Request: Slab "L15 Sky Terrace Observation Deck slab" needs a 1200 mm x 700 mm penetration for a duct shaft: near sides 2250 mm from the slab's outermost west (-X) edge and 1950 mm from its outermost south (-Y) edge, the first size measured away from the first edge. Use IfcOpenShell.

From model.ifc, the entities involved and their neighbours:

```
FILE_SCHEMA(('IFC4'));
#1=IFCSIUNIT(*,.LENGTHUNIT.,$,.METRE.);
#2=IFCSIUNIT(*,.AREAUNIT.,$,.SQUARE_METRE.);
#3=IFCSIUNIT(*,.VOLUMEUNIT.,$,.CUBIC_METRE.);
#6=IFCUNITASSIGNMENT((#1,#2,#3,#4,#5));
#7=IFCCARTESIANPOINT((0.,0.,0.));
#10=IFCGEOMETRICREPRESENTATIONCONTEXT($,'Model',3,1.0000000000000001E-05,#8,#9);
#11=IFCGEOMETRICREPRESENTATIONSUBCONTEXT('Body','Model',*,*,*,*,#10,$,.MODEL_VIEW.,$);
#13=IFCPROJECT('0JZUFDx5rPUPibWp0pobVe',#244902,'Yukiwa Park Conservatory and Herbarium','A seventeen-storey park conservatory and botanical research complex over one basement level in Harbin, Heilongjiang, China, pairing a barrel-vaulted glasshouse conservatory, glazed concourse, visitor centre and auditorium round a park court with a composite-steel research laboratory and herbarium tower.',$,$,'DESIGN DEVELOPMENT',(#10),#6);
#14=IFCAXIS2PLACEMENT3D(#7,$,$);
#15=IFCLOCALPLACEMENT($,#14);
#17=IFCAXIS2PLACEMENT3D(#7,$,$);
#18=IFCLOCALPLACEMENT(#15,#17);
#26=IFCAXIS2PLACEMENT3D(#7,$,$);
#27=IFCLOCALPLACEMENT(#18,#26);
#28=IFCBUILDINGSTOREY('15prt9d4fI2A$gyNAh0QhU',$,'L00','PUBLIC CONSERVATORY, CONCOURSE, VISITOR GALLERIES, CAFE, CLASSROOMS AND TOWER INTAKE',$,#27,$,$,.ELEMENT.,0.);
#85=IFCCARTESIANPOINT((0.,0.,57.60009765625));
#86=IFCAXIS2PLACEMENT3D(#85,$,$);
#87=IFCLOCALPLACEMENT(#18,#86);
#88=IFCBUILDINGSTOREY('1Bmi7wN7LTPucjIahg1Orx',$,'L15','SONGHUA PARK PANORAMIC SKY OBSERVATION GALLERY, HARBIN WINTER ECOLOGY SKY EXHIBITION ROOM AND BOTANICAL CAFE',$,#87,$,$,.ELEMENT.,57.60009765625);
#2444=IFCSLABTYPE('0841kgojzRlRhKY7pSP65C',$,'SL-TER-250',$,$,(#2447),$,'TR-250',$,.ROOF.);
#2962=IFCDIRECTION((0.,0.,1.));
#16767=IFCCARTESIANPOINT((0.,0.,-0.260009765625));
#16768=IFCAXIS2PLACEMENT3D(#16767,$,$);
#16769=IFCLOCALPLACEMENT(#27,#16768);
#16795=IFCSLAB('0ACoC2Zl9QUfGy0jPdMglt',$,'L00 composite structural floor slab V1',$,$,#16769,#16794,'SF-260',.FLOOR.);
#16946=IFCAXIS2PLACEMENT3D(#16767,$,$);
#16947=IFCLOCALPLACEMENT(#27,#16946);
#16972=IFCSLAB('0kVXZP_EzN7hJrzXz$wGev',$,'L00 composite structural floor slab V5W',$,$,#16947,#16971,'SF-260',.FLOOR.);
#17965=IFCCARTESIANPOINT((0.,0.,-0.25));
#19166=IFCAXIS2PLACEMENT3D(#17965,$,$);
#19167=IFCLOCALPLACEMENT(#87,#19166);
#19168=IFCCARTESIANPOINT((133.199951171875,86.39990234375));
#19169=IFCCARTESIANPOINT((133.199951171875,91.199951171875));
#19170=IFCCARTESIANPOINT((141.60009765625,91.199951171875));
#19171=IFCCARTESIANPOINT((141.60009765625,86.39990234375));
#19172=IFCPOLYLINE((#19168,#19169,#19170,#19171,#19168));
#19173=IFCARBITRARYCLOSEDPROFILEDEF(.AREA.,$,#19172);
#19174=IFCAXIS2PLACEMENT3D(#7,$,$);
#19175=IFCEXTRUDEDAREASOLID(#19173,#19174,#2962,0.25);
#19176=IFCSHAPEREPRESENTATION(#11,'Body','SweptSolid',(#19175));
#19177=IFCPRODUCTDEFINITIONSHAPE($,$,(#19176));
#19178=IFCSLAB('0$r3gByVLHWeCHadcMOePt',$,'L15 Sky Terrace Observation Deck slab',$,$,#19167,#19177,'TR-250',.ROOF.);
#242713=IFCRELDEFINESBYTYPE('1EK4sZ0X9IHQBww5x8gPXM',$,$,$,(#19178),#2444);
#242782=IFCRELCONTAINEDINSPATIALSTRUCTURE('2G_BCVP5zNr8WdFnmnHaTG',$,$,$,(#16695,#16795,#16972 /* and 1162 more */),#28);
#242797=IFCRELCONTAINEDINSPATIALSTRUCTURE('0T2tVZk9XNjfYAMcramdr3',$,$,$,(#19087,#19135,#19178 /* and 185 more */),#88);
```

```python
import numpy as np
import ifcopenshell
import ifcopenshell.api.feature
import ifcopenshell.api.geometry
import ifcopenshell.api.root
import ifcopenshell.geom
import ifcopenshell.util.placement
import ifcopenshell.util.representation
import ifcopenshell.util.shape
import ifcopenshell.util.unit

model = ifcopenshell.open("model.ifc")
unit_scale = ifcopenshell.util.unit.calculate_unit_scale(model)
settings = ifcopenshell.geom.settings()


def volume(element):
    """Net volume in cubic metres, openings subtracted."""
    shape = ifcopenshell.geom.create_shape(settings, element)
    return ifcopenshell.util.shape.get_volume(shape.geometry)


slab = model.by_id(19178)
before = volume(slab)

# Extent in the slab's own axes, in metres. The edges named are its -X and -Y sides.
slab_shape = ifcopenshell.geom.create_shape(settings, slab)
vertices = ifcopenshell.util.shape.get_vertices(slab_shape.geometry)
x_min, y_min, bottom = vertices.min(axis=0)
top = vertices[:, 2].max()

opening = ifcopenshell.api.root.create_entity(model, ifc_class="IfcOpeningElement", name="Duct shaft opening", predefined_type="OPENING")
context = ifcopenshell.util.representation.get_context(model, "Model", "Body", "MODEL_VIEW")
width, depth = 1.2, 0.7
outline = [(0.0, 0.0), (width, 0.0), (width, depth), (0.0, depth), (0.0, 0.0)]
# Overshoot both faces by 50 mm so the cut is clean.
shape = ifcopenshell.api.geometry.add_slab_representation(
    model, context=context, depth=top - bottom + 0.1, polyline=outline
)
ifcopenshell.api.geometry.assign_representation(model, product=opening, representation=shape)

matrix = ifcopenshell.util.placement.get_local_placement(slab.ObjectPlacement)
matrix[:, 3] = matrix @ np.append(np.array([x_min + 2.25, y_min + 1.95, bottom - 0.05]) / unit_scale, 1.0)
ifcopenshell.api.geometry.edit_object_placement(model, product=opening, matrix=matrix, is_si=False)
ifcopenshell.api.feature.add_feature(model, feature=opening, element=slab)

after = volume(slab)

print(f"slab volume {before:.3f} -> {after:.3f} m3")

model.write("model_edited.ifc")
```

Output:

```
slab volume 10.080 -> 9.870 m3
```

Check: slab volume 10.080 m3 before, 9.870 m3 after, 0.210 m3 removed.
